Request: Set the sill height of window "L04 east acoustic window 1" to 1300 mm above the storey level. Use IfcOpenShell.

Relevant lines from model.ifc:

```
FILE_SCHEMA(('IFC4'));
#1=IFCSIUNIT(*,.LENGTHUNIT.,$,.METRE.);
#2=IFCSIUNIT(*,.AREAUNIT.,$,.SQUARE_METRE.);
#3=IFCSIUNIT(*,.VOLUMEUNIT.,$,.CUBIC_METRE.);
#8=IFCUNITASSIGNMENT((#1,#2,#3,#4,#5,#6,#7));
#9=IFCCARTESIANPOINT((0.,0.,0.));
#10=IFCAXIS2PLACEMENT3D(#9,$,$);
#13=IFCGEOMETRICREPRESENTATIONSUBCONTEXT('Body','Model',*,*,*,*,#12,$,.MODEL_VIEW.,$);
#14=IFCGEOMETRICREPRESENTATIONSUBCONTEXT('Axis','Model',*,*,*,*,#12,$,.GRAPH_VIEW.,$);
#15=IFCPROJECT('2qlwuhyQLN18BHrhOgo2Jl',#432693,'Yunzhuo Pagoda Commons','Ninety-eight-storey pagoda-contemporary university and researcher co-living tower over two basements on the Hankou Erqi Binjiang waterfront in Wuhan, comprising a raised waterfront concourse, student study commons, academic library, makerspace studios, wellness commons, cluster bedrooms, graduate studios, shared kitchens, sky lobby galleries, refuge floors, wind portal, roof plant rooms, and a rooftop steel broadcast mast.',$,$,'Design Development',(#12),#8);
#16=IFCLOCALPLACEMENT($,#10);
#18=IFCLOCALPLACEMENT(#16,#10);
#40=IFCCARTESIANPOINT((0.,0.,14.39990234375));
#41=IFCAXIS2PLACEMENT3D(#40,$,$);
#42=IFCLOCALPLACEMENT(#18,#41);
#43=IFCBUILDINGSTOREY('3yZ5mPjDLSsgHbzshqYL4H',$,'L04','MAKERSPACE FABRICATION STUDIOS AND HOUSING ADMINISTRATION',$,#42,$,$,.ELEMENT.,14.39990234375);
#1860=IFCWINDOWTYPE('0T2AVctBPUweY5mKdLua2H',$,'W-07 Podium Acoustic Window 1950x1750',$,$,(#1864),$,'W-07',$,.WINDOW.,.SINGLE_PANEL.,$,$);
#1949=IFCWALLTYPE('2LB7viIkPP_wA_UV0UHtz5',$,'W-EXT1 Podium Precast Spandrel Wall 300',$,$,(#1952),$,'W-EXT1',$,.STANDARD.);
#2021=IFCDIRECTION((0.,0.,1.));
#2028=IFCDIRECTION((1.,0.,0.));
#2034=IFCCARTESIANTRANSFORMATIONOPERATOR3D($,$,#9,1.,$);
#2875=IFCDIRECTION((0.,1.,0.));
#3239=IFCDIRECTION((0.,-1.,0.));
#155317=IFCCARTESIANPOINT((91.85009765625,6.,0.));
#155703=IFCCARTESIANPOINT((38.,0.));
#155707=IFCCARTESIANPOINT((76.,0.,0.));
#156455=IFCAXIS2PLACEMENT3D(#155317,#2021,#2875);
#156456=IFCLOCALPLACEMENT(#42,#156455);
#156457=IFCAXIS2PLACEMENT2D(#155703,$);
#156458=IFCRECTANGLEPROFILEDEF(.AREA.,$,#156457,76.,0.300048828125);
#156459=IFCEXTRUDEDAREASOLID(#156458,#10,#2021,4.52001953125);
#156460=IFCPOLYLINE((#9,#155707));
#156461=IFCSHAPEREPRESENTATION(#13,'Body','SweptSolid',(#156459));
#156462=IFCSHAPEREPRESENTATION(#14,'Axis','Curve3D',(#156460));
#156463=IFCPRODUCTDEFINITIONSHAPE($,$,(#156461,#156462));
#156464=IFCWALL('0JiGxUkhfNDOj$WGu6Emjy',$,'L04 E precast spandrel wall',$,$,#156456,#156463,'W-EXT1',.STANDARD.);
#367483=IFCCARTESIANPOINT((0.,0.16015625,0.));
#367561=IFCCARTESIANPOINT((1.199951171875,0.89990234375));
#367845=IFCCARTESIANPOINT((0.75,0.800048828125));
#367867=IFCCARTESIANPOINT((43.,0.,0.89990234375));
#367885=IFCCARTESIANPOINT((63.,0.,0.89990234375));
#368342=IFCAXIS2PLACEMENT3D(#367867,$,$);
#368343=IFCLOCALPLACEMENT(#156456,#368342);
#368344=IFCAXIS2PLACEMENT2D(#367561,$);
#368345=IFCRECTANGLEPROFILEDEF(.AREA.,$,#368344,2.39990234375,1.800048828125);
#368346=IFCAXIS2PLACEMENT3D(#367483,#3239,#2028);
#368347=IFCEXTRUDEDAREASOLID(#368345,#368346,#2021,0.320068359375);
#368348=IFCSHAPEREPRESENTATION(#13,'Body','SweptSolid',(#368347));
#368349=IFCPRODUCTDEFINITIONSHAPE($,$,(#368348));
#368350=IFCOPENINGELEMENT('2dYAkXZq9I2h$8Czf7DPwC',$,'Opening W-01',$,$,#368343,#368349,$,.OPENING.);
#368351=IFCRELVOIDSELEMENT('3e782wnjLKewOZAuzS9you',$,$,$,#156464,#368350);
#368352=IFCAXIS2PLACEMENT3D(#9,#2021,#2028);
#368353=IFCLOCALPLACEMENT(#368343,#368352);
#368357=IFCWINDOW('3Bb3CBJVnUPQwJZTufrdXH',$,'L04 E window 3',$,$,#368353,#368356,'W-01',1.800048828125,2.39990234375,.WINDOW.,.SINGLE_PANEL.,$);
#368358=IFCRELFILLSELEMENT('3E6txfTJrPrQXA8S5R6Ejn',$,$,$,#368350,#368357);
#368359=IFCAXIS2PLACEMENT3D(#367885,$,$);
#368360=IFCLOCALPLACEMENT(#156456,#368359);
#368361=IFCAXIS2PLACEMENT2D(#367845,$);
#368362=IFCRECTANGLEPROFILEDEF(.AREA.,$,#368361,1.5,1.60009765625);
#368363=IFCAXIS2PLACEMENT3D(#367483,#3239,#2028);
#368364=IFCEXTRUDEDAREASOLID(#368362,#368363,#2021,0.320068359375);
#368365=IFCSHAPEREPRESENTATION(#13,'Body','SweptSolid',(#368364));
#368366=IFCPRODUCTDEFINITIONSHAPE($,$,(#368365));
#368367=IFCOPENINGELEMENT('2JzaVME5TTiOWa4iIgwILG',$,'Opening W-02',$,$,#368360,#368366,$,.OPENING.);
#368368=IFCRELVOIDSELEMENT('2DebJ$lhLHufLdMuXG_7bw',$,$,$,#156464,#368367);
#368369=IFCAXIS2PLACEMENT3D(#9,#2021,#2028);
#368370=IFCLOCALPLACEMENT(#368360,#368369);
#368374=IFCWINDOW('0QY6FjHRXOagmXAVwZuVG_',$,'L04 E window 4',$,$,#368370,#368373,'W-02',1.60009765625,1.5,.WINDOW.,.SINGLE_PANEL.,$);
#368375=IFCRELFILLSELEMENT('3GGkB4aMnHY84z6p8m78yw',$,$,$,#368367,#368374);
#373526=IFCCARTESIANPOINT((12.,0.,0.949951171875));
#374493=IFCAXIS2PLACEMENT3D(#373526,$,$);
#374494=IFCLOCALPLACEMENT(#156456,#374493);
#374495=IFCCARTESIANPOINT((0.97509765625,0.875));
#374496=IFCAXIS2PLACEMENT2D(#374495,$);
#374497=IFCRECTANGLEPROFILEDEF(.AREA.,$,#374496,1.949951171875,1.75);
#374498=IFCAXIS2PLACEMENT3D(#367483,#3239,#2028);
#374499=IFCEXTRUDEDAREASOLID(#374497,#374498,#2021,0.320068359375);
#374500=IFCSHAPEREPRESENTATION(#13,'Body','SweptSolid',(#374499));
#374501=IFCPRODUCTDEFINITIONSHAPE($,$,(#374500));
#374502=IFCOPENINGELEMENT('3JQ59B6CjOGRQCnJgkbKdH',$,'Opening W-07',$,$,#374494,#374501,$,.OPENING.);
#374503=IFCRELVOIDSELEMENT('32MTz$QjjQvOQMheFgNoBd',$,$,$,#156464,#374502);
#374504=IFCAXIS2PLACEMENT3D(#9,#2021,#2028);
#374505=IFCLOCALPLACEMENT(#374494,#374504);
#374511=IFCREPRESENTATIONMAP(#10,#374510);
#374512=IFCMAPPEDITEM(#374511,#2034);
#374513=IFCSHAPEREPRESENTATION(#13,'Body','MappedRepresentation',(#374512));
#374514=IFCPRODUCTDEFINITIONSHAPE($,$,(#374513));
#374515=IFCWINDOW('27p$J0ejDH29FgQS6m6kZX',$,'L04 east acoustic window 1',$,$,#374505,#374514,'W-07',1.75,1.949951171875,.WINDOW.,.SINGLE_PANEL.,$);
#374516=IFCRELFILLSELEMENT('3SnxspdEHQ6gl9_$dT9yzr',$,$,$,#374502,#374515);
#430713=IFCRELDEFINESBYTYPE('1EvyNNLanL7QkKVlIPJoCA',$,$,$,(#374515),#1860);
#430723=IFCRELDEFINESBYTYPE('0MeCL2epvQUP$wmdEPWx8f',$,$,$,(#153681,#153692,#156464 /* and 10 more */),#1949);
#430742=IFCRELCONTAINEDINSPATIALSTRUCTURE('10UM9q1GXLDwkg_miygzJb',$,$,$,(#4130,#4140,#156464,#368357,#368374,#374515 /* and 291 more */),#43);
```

```python
import numpy as np
import ifcopenshell
import ifcopenshell.api.geometry
import ifcopenshell.geom
import ifcopenshell.util.element
import ifcopenshell.util.placement
import ifcopenshell.util.shape
import ifcopenshell.util.unit

model = ifcopenshell.open("model.ifc")
unit_scale = ifcopenshell.util.unit.calculate_unit_scale(model)

window = model.by_guid("27p$J0ejDH29FgQS6m6kZX")
opening = window.FillsVoids[0].RelatingOpeningElement
storey = ifcopenshell.util.element.get_container(window, ifc_class="IfcBuildingStorey")
level = ifcopenshell.util.placement.get_local_placement(storey.ObjectPlacement)[2, 3]

# The opening's origin need not be at the sill, so measure its lowest point.
shape = ifcopenshell.geom.create_shape(ifcopenshell.geom.settings(), opening)
bottom = ifcopenshell.util.shape.get_shape_bottom_elevation(shape, shape.geometry) / unit_scale
dz = level + 1.3 / unit_scale - bottom

shift = np.array([0.0, 0.0, dz])
# The window is placed relative to its opening, so it follows when the opening moves.
matrix = ifcopenshell.util.placement.get_local_placement(opening.ObjectPlacement)
matrix[:3, 3] += shift
ifcopenshell.api.geometry.edit_object_placement(
    model, product=opening, matrix=matrix, is_si=False, should_transform_children=True
)

print(f"moved by {dz * unit_scale:+.3f} m")

model.write("model-out.ifc")
```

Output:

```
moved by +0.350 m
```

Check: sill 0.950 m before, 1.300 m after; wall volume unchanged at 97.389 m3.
